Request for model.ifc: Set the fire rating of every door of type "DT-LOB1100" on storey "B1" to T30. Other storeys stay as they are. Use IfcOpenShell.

First a look at what the model holds.

```python
import ifcopenshell
import ifcopenshell.util.element

model = ifcopenshell.open("model.ifc")
print(model.schema)
storey = next(s for s in model.by_type("IfcBuildingStorey") if s.Name == "B1")
doors = [e for e in ifcopenshell.util.element.get_decomposition(storey) if e.is_a("IfcDoor")]
seen = {}
for e in doors:
    element_type = ifcopenshell.util.element.get_type(e)
    key = (element_type.Name if element_type != e and element_type else None, ifcopenshell.util.element.get_pset(e, "Pset_DoorCommon", "FireRating"))
    seen[key] = seen.get(key, 0) + 1
for (name, value), count in sorted(seen.items(), key=str):
    print(count, "x", name, "|", value)
```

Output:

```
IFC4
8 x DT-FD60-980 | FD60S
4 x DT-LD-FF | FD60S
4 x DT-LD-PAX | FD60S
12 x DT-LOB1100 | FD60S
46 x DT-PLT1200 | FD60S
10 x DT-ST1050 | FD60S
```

```python
import ifcopenshell
import ifcopenshell.api.pset
import ifcopenshell.util.element

model = ifcopenshell.open("model.ifc")

storey = next(s for s in model.by_type("IfcBuildingStorey") if s.Name == "B1")
doors = [e for e in ifcopenshell.util.element.get_decomposition(storey) if e.is_a("IfcDoor")]

count = 0
for e in doors:
    element_type = ifcopenshell.util.element.get_type(e)
    if element_type in (None, e) or element_type.Name != "DT-LOB1100":
        continue
    # add_pset returns the element's existing set when there is one.
    pset = ifcopenshell.api.pset.add_pset(model, product=e, name="Pset_DoorCommon")
    ifcopenshell.api.pset.edit_pset(model, pset=pset, properties={"FireRating": "T30"})
    count += 1

print(count, "doors updated")

model.write("model-out.ifc")
```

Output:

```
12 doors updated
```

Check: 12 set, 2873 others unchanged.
